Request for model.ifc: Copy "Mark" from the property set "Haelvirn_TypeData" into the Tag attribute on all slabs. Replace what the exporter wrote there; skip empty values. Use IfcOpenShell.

First a look at what the model holds.

```python
import ifcopenshell
import ifcopenshell.util.element

model = ifcopenshell.open("model.ifc")
print(model.schema)
slabs = model.by_type("IfcSlab")
print(len(slabs), "slabs")
for e in slabs[:8]:
    source = ifcopenshell.util.element.get_pset(e, "Haelvirn_TypeData", "Mark")
    target = e.Tag
    print(e.id(), repr(source), repr(target), sep=" | ")
```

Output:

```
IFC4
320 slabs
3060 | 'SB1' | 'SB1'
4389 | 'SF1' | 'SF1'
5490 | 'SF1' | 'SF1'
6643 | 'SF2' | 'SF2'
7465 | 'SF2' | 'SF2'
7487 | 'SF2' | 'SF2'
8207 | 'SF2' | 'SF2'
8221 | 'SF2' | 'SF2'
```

```python
import ifcopenshell
import ifcopenshell.util.element

model = ifcopenshell.open("model.ifc")

count = 0
for e in model.by_type("IfcSlab"):
    value = ifcopenshell.util.element.get_pset(e, "Haelvirn_TypeData", "Mark")
    current = e.Tag
    if not value or not value.strip() or current == value:
        continue
    e.Tag = value
    count += 1

print(count, "slabs updated")

model.write("model-out.ifc")
```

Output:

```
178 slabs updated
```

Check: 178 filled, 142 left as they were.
